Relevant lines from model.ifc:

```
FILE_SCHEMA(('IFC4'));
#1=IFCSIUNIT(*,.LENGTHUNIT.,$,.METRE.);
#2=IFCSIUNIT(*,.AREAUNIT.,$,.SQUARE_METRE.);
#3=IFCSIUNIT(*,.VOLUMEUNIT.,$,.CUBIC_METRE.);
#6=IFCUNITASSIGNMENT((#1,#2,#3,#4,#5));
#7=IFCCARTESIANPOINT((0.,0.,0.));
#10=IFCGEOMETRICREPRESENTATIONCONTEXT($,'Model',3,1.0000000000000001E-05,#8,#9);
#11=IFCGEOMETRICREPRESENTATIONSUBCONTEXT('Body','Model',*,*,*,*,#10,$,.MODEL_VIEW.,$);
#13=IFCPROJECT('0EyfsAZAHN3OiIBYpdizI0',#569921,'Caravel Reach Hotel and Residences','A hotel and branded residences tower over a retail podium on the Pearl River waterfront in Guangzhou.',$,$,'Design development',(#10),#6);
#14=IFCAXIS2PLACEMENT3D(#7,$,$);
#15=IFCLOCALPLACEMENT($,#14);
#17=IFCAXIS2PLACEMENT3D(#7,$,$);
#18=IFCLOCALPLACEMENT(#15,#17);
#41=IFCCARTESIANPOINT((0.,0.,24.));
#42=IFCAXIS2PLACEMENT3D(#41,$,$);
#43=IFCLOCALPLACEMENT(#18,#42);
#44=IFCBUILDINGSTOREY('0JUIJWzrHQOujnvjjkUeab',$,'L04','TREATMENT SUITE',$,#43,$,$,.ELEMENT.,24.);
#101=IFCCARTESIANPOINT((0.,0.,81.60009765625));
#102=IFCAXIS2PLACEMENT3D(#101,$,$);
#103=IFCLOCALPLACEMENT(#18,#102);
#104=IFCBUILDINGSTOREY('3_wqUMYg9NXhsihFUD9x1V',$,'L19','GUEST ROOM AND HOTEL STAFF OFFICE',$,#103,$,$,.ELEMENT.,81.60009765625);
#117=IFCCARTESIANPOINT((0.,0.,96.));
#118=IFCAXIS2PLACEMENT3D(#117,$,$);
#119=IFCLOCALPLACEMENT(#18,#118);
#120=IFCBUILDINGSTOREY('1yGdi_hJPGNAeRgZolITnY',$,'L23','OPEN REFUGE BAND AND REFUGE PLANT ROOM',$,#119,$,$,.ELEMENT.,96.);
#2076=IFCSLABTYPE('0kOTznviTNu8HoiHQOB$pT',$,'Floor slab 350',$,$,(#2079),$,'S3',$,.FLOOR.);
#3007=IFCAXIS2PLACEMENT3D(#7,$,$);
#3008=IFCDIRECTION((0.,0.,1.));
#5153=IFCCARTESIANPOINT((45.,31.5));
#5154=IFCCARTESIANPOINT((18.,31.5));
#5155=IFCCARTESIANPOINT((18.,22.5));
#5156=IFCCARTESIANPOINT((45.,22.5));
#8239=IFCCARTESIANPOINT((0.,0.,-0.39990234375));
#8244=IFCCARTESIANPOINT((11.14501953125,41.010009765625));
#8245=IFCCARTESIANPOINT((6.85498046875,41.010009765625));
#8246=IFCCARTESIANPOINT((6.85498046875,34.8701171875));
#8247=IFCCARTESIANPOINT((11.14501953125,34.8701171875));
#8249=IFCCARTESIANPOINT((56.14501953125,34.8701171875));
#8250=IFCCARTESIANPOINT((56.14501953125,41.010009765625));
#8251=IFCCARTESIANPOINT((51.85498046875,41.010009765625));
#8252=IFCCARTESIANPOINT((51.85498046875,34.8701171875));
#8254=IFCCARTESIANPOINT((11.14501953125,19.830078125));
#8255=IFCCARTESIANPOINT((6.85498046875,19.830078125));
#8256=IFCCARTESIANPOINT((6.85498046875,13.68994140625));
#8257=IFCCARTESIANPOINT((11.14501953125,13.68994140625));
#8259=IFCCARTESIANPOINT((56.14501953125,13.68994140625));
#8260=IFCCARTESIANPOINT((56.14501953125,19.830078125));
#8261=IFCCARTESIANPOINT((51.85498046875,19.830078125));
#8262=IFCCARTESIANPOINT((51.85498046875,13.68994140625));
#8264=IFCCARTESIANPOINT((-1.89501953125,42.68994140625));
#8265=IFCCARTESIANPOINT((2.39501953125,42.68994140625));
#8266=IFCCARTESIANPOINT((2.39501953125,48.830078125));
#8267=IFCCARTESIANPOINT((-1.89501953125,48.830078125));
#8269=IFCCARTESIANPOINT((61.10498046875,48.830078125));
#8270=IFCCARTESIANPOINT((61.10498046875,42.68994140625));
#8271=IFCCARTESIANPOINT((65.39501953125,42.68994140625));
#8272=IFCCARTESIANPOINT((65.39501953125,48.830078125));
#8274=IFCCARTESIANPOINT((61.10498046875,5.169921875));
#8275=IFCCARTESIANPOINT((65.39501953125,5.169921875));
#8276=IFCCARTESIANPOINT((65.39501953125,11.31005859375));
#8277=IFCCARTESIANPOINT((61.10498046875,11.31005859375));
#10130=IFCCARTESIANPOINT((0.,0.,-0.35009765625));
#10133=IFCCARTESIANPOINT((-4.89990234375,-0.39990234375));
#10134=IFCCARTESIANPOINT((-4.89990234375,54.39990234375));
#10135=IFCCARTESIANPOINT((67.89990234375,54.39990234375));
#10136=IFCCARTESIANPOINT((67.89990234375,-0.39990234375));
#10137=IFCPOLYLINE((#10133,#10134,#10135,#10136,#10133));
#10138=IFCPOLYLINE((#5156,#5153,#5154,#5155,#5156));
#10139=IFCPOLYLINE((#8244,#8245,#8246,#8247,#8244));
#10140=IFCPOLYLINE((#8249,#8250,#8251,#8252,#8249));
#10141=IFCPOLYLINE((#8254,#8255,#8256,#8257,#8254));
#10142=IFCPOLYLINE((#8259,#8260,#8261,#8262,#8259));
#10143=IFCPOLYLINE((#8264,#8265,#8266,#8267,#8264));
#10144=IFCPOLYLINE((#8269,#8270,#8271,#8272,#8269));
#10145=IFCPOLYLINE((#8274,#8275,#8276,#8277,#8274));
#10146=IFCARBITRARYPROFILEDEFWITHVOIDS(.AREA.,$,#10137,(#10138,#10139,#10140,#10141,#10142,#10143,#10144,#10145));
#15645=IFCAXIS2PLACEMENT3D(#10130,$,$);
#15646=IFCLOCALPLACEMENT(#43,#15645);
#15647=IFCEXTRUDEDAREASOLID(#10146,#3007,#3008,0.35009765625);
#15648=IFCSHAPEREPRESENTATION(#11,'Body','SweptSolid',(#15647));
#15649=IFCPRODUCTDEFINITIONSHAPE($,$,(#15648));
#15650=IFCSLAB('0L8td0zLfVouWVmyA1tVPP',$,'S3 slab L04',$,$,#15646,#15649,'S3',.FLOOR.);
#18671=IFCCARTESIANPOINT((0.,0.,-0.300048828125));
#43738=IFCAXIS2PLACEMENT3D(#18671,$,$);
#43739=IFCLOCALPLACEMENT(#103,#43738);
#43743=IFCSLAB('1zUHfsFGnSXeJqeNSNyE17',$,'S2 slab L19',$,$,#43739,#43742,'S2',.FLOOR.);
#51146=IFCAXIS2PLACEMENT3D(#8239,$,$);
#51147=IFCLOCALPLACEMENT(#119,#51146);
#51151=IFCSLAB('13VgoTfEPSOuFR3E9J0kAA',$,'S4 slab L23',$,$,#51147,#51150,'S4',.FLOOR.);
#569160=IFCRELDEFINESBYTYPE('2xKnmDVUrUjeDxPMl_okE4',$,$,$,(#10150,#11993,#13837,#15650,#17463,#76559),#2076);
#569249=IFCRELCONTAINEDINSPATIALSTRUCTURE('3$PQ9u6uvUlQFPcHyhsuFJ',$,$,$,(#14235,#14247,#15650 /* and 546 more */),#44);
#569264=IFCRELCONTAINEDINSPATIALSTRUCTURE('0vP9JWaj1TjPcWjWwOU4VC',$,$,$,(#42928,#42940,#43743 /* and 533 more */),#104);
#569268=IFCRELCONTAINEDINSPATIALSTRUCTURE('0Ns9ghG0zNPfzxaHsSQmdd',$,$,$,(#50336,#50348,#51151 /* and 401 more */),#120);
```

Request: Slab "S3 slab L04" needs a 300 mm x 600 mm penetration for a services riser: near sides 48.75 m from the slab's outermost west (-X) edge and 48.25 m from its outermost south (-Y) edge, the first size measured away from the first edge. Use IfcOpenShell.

```python
import numpy as np
import ifcopenshell
import ifcopenshell.api.feature
import ifcopenshell.api.geometry
import ifcopenshell.api.root
import ifcopenshell.geom
import ifcopenshell.util.placement
import ifcopenshell.util.representation
import ifcopenshell.util.shape
import ifcopenshell.util.unit

model = ifcopenshell.open("model.ifc")
unit_scale = ifcopenshell.util.unit.calculate_unit_scale(model)
settings = ifcopenshell.geom.settings()


def volume(element):
    """Net volume in cubic metres, openings subtracted."""
    shape = ifcopenshell.geom.create_shape(settings, element)
    return ifcopenshell.util.shape.get_volume(shape.geometry)


slab = model.by_guid("0L8td0zLfVouWVmyA1tVPP")
before = volume(slab)

# Extent in the slab's own axes, in metres. The edges named are its -X and -Y sides.
slab_shape = ifcopenshell.geom.create_shape(settings, slab)
vertices = ifcopenshell.util.shape.get_vertices(slab_shape.geometry)
x_min, y_min, bottom = vertices.min(axis=0)
top = vertices[:, 2].max()

opening = ifcopenshell.api.root.create_entity(model, ifc_class="IfcOpeningElement", name="Services riser opening", predefined_type="OPENING")
context = ifcopenshell.util.representation.get_context(model, "Model", "Body", "MODEL_VIEW")
width, depth = 0.3, 0.6
outline = [(0.0, 0.0), (width, 0.0), (width, depth), (0.0, depth), (0.0, 0.0)]
# Overshoot both faces by 50 mm so the cut is clean.
shape = ifcopenshell.api.geometry.add_slab_representation(
    model, context=context, depth=top - bottom + 0.1, polyline=outline
)
ifcopenshell.api.geometry.assign_representation(model, product=opening, representation=shape)

matrix = ifcopenshell.util.placement.get_local_placement(slab.ObjectPlacement)
matrix[:, 3] = matrix @ np.append(np.array([x_min + 48.75, y_min + 48.25, bottom - 0.05]) / unit_scale, 1.0)
ifcopenshell.api.geometry.edit_object_placement(model, product=opening, matrix=matrix, is_si=False)
ifcopenshell.api.feature.add_feature(model, feature=opening, element=slab)

after = volume(slab)

print(f"slab volume {before:.3f} -> {after:.3f} m3")

model.write("model_updated.ifc")
```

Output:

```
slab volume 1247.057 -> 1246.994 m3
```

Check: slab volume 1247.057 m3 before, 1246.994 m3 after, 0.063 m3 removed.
